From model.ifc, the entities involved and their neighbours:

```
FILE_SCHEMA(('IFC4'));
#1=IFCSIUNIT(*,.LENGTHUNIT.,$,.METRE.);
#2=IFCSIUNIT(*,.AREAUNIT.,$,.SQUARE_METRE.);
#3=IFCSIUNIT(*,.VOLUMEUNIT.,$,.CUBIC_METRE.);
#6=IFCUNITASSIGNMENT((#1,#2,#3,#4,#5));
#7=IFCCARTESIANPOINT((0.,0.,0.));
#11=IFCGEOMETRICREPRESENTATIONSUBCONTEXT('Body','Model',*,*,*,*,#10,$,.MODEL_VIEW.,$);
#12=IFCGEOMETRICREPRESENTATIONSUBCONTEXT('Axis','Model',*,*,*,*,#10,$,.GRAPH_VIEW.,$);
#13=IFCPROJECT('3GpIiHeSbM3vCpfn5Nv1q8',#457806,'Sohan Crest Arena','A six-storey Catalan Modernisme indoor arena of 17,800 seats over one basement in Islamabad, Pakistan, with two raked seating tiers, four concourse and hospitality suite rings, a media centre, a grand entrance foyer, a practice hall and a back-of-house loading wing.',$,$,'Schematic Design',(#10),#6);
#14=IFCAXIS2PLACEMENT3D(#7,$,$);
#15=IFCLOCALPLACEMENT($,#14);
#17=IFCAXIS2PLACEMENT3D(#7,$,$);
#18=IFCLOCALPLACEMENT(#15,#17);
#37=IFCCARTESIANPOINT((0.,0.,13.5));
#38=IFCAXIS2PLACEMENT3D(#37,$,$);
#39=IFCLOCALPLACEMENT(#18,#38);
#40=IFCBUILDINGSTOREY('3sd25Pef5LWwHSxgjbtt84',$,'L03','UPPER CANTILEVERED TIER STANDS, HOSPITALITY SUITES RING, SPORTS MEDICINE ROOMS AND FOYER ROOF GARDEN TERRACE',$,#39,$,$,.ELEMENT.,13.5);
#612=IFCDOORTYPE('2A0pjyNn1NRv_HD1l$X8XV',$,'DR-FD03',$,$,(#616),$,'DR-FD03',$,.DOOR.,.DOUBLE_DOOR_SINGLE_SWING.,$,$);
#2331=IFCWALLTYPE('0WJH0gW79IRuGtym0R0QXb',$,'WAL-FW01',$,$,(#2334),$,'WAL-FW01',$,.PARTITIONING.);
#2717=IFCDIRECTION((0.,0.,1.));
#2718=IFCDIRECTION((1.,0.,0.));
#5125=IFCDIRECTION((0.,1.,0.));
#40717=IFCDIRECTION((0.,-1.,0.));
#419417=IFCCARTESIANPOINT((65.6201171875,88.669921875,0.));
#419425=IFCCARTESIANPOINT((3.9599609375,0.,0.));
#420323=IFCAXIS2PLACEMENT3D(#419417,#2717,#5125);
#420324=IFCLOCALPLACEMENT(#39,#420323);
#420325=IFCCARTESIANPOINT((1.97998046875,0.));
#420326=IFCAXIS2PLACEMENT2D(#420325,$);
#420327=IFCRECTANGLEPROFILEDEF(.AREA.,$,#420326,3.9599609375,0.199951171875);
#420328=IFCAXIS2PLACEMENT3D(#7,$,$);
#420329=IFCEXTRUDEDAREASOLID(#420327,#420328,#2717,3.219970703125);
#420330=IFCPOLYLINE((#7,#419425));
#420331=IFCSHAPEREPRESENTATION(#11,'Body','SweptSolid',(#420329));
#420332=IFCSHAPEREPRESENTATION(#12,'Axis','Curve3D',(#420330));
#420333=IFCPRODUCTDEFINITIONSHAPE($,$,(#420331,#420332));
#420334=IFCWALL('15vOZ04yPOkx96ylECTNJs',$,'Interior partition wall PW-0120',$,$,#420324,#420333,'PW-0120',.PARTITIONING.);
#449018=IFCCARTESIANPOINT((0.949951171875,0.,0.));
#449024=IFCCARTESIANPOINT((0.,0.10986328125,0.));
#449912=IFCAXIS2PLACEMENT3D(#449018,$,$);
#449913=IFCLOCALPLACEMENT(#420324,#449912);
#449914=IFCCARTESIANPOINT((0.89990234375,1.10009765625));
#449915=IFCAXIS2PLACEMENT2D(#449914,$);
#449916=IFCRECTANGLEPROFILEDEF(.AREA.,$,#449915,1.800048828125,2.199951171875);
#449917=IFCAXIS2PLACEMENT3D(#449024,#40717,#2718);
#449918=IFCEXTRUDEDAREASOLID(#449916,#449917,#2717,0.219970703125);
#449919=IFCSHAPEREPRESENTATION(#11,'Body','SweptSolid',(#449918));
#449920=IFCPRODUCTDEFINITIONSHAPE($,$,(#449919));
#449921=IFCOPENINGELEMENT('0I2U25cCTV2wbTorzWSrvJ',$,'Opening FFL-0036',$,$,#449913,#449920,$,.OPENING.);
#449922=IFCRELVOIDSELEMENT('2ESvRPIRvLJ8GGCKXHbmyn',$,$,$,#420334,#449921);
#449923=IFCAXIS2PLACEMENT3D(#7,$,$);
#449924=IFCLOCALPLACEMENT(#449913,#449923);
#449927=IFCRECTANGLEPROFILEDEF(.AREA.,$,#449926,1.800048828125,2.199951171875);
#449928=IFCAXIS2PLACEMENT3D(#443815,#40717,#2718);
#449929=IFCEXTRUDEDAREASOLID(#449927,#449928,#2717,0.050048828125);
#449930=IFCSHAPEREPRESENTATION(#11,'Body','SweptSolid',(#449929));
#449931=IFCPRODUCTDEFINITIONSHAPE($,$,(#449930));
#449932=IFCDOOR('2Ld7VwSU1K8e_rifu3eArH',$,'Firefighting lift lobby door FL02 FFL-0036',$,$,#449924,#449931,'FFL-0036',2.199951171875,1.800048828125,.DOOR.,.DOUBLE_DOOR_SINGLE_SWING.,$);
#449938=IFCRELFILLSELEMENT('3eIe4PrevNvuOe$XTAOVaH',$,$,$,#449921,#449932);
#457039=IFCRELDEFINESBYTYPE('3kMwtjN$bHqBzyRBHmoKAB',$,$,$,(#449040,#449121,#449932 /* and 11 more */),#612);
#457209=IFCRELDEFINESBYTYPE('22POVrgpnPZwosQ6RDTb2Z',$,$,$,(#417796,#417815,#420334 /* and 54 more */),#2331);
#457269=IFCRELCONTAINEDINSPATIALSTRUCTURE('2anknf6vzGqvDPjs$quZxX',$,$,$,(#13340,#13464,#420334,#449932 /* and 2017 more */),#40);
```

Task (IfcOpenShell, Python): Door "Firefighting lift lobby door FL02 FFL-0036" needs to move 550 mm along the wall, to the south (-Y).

```python
import ifcopenshell
import ifcopenshell.api.geometry
import ifcopenshell.util.placement

model = ifcopenshell.open("model.ifc")

door = model.by_guid("2Ld7VwSU1K8e_rifu3eArH")
opening = door.FillsVoids[0].RelatingOpeningElement
wall = opening.VoidsElements[0].RelatingBuildingElement

wall_matrix = ifcopenshell.util.placement.get_local_placement(wall.ObjectPlacement)
shift = wall_matrix[:3, 0] * -0.55
before = ifcopenshell.util.placement.get_local_placement(door.ObjectPlacement)[:3, 3].copy()

# The door is placed relative to its opening, so it follows when the opening moves.
matrix = ifcopenshell.util.placement.get_local_placement(opening.ObjectPlacement)
matrix[:3, 3] += shift
ifcopenshell.api.geometry.edit_object_placement(
    model, product=opening, matrix=matrix, is_si=False, should_transform_children=True
)

after = ifcopenshell.util.placement.get_local_placement(door.ObjectPlacement)[:3, 3]
print("door moved by", (after - before).round(3) + 0.0)

model.write("model_v2.ifc")
```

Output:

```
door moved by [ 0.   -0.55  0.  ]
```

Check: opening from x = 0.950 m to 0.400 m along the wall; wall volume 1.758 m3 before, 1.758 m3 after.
